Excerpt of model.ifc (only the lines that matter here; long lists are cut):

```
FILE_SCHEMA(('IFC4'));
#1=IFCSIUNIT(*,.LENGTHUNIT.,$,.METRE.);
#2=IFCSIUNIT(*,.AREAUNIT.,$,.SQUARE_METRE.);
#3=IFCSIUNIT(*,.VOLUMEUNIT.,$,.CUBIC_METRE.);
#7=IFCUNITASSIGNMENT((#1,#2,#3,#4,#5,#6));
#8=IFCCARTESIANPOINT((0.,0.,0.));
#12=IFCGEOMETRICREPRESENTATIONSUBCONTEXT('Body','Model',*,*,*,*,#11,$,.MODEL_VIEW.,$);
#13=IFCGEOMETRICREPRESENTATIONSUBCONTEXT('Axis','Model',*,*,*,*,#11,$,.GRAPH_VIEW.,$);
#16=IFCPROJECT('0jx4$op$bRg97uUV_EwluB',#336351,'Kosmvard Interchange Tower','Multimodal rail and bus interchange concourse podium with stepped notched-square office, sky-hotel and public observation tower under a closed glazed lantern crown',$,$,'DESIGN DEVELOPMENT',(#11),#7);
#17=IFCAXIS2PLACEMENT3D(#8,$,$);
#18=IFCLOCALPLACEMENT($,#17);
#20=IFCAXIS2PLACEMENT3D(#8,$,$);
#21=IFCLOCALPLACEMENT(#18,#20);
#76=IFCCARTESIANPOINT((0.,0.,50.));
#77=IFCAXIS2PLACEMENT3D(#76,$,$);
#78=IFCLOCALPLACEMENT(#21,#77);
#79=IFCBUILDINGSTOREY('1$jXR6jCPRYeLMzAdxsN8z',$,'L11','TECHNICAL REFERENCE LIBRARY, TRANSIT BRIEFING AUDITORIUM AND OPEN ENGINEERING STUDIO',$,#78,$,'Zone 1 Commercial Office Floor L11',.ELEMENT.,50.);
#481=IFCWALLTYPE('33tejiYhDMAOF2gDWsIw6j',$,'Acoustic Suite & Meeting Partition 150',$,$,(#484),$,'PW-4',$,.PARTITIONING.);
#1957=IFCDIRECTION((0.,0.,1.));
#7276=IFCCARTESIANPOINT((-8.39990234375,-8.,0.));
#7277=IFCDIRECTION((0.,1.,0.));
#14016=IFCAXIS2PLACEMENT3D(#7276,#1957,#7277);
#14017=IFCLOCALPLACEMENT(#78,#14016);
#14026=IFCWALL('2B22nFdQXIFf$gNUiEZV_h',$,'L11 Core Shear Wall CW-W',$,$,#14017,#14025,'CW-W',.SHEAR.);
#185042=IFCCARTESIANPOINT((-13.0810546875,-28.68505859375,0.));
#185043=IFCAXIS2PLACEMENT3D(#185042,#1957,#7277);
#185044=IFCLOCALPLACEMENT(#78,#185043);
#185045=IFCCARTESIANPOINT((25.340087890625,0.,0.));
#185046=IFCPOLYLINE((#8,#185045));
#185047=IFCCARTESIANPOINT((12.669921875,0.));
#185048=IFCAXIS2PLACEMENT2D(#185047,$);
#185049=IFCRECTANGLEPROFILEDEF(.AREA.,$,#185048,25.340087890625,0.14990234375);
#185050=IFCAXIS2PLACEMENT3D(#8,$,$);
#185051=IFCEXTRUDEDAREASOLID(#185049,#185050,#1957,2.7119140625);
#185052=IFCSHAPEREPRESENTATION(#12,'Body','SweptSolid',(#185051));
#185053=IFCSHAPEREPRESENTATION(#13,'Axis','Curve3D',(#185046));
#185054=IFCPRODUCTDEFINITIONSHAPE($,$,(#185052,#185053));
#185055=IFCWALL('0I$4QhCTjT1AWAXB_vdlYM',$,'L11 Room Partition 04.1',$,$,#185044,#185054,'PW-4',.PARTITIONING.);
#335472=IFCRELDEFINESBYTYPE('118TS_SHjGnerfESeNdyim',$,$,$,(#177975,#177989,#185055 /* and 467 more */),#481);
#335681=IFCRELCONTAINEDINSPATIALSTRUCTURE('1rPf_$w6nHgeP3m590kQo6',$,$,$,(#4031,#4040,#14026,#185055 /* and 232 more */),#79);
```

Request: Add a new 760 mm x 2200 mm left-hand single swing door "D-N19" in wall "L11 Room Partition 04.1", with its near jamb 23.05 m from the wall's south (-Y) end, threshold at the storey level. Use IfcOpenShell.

```python
import numpy as np
import ifcopenshell
import ifcopenshell.api.feature
import ifcopenshell.api.geometry
import ifcopenshell.api.root
import ifcopenshell.api.spatial
import ifcopenshell.geom
import ifcopenshell.util.element
import ifcopenshell.util.placement
import ifcopenshell.util.representation
import ifcopenshell.util.shape
import ifcopenshell.util.unit

model = ifcopenshell.open("model.ifc")
unit_scale = ifcopenshell.util.unit.calculate_unit_scale(model)
settings = ifcopenshell.geom.settings()


def volume(element):
    """Net volume in cubic metres, openings subtracted."""
    shape = ifcopenshell.geom.create_shape(settings, element)
    return ifcopenshell.util.shape.get_volume(shape.geometry)


wall = model.by_guid("0I$4QhCTjT1AWAXB_vdlYM")
storey = ifcopenshell.util.element.get_container(wall, ifc_class="IfcBuildingStorey")
context = ifcopenshell.util.representation.get_context(model, "Model", "Body", "MODEL_VIEW")
before = volume(wall)

width, height, from_end, sill = 0.76, 2.2, 23.05, 0.0  # metres

# The wall runs along its own X axis, and the end named is its -X end.
wall_shape = ifcopenshell.geom.create_shape(settings, wall)
x, y, z = ifcopenshell.util.shape.get_vertices(wall_shape.geometry).T
start = x.min() + from_end
face, thickness = float(y.min()), float(y.max() - y.min())
wall_matrix = ifcopenshell.util.placement.get_local_placement(wall.ObjectPlacement)
level = ifcopenshell.util.placement.get_local_placement(storey.ObjectPlacement)[2, 3]


def in_wall(x, y):
    """Placement at x, y metres in the wall's axes, at sill height."""
    matrix = wall_matrix.copy()
    matrix[:, 3] = wall_matrix @ np.array([x / unit_scale, y / unit_scale, 0.0, 1.0])
    matrix[2, 3] = level + sill / unit_scale
    return matrix


# Opening: a box that overshoots both wall faces by 50 mm.
opening = ifcopenshell.api.root.create_entity(model, ifc_class="IfcOpeningElement", predefined_type="OPENING")
box = ifcopenshell.api.geometry.add_wall_representation(
    model, context=context, length=width, height=height, thickness=thickness + 0.1
)
ifcopenshell.api.geometry.assign_representation(model, product=opening, representation=box)
ifcopenshell.api.geometry.edit_object_placement(model, product=opening, matrix=in_wall(start, face - 0.05), is_si=False)
ifcopenshell.api.feature.add_feature(model, feature=opening, element=wall)

door = ifcopenshell.api.root.create_entity(model, ifc_class="IfcDoor", name="D-N19", predefined_type="DOOR")
door.OverallWidth, door.OverallHeight = width / unit_scale, height / unit_scale
door.OperationType = "SINGLE_SWING_LEFT"
body = ifcopenshell.api.geometry.add_door_representation(
    model,
    context=context,
    overall_width=door.OverallWidth,
    overall_height=door.OverallHeight,
    operation_type="SINGLE_SWING_LEFT",
    lining_properties={"LiningDepth": thickness / unit_scale, "ThresholdDepth": thickness / unit_scale},
)
ifcopenshell.api.geometry.assign_representation(model, product=door, representation=body)
ifcopenshell.api.spatial.assign_container(model, products=[door], relating_structure=storey)
ifcopenshell.api.feature.add_filling(model, opening=opening, element=door)

# The lining spans the wall, so the door starts at the wall face.
ifcopenshell.api.geometry.edit_object_placement(model, product=door, matrix=in_wall(start, face), is_si=False)

after = volume(wall)

print(f"wall volume {before:.3f} -> {after:.3f} m3")

model.write("model_v2.ifc")
```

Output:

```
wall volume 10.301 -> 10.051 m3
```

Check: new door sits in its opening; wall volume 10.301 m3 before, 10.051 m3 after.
